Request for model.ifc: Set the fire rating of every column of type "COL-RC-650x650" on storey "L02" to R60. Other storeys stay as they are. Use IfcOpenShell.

First a look at what the model holds.

```python
import ifcopenshell
import ifcopenshell.util.element

model = ifcopenshell.open("model.ifc")
print(model.schema)
storey = next(s for s in model.by_type("IfcBuildingStorey") if s.Name == "L02")
columns = [e for e in ifcopenshell.util.element.get_decomposition(storey) if e.is_a("IfcColumn")]
seen = {}
for e in columns:
    element_type = ifcopenshell.util.element.get_type(e)
    key = (element_type.Name if element_type != e and element_type else None, ifcopenshell.util.element.get_pset(e, "Pset_ColumnCommon", "FireRating"))
    seen[key] = seen.get(key, 0) + 1
for (name, value), count in sorted(seen.items(), key=str):
    print(count, "x", name, "|", value)
```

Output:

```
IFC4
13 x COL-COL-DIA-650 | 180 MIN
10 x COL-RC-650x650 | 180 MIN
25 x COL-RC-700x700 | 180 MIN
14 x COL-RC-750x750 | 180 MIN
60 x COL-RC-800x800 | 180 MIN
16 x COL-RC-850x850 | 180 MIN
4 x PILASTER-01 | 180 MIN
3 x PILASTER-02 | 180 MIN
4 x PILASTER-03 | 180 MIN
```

```python
import ifcopenshell
import ifcopenshell.api.pset
import ifcopenshell.util.element

model = ifcopenshell.open("model.ifc")

storey = next(s for s in model.by_type("IfcBuildingStorey") if s.Name == "L02")
columns = [e for e in ifcopenshell.util.element.get_decomposition(storey) if e.is_a("IfcColumn")]

count = 0
for e in columns:
    element_type = ifcopenshell.util.element.get_type(e)
    if element_type in (None, e) or element_type.Name != "COL-RC-650x650":
        continue
    # add_pset returns the element's existing set when there is one.
    pset = ifcopenshell.api.pset.add_pset(model, product=e, name="Pset_ColumnCommon")
    ifcopenshell.api.pset.edit_pset(model, pset=pset, properties={"FireRating": "R60"})
    count += 1

print(count, "columns updated")

model.write("model_v2.ifc")
```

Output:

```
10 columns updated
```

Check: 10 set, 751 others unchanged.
